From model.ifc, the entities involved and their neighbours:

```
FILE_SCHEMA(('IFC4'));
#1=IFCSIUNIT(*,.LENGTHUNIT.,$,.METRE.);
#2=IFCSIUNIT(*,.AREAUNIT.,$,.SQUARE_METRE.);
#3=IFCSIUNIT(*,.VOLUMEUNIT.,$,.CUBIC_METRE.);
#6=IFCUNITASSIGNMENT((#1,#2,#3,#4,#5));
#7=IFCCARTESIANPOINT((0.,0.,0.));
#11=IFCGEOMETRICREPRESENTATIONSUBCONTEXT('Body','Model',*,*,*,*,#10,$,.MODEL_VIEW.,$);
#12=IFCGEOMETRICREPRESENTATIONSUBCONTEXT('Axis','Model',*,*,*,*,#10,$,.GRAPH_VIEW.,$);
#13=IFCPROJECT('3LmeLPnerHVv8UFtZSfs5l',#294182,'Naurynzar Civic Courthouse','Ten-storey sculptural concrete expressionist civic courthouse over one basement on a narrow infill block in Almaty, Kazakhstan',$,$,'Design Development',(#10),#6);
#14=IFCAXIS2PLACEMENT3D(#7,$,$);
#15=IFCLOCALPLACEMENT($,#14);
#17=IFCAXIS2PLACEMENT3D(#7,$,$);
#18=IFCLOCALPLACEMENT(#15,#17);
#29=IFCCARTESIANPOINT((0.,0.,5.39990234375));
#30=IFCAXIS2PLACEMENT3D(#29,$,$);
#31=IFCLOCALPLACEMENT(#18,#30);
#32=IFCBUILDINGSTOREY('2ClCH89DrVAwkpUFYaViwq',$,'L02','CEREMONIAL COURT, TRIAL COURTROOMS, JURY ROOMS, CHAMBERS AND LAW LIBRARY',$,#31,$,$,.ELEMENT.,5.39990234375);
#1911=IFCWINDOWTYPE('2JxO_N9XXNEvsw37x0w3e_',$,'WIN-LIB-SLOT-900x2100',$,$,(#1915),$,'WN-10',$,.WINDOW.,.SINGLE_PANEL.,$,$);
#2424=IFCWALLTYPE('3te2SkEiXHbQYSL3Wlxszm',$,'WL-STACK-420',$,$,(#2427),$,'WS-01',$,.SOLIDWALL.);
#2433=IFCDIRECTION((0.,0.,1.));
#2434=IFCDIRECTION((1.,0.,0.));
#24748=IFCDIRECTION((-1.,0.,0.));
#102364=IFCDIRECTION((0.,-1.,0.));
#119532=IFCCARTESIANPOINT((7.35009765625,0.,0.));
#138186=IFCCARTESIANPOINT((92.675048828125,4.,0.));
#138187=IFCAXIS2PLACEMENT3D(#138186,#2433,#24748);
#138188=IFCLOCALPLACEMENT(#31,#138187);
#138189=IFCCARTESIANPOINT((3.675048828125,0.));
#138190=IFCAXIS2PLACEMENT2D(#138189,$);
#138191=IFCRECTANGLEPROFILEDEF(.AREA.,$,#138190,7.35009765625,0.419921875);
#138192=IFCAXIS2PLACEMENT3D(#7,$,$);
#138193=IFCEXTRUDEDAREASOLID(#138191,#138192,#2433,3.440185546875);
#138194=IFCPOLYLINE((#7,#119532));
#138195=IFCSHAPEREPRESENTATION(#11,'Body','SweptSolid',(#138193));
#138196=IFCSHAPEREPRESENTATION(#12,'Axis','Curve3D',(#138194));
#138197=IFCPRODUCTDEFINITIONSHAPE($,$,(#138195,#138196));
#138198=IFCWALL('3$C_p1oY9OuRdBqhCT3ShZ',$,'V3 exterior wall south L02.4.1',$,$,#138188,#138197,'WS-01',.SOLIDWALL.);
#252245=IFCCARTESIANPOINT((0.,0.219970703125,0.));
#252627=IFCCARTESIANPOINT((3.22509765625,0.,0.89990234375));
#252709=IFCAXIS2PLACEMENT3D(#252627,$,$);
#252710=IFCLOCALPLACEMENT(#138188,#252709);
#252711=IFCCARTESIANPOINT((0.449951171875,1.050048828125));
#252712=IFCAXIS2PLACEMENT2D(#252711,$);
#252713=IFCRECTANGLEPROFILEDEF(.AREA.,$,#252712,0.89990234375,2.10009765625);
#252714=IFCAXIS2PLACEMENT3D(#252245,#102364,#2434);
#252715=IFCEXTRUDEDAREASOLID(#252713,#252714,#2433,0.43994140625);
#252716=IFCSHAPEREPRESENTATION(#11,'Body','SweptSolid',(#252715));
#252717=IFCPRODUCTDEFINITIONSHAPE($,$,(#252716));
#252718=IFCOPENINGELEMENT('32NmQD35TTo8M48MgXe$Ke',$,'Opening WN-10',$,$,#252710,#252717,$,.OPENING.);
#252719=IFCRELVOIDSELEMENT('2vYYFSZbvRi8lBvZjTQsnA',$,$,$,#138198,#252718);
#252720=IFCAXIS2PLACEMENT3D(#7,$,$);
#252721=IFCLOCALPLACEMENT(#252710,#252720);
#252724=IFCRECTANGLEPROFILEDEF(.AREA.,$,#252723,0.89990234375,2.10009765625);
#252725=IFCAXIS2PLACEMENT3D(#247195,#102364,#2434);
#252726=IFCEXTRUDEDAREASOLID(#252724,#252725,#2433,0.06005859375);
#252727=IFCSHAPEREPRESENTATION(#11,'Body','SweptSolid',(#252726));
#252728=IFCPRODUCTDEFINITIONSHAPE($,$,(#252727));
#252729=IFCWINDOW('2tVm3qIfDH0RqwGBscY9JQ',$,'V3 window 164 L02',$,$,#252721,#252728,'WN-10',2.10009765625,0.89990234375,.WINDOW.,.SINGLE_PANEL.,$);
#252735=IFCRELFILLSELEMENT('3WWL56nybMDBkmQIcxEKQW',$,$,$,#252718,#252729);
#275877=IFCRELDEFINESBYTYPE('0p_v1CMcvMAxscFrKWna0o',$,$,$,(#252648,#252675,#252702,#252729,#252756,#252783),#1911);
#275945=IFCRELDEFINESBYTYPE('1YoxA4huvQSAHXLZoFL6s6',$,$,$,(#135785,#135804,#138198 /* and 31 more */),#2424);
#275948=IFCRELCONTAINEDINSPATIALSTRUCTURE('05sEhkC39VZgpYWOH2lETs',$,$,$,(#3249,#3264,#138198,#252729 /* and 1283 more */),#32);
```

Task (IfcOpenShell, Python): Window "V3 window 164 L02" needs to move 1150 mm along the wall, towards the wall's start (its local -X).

```python
import ifcopenshell
import ifcopenshell.api.geometry
import ifcopenshell.util.placement

model = ifcopenshell.open("model.ifc")

window = model.by_guid("2tVm3qIfDH0RqwGBscY9JQ")
opening = window.FillsVoids[0].RelatingOpeningElement
wall = opening.VoidsElements[0].RelatingBuildingElement

wall_matrix = ifcopenshell.util.placement.get_local_placement(wall.ObjectPlacement)
shift = wall_matrix[:3, 0] * -1.15
before = ifcopenshell.util.placement.get_local_placement(window.ObjectPlacement)[:3, 3].copy()

# The window is placed relative to its opening, so it follows when the opening moves.
matrix = ifcopenshell.util.placement.get_local_placement(opening.ObjectPlacement)
matrix[:3, 3] += shift
ifcopenshell.api.geometry.edit_object_placement(
    model, product=opening, matrix=matrix, is_si=False, should_transform_children=True
)

after = ifcopenshell.util.placement.get_local_placement(window.ObjectPlacement)[:3, 3]
print("window moved by", (after - before).round(3) + 0.0)

model.write("model_rev.ifc")
```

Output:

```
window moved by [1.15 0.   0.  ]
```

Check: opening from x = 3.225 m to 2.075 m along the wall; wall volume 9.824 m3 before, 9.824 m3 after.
